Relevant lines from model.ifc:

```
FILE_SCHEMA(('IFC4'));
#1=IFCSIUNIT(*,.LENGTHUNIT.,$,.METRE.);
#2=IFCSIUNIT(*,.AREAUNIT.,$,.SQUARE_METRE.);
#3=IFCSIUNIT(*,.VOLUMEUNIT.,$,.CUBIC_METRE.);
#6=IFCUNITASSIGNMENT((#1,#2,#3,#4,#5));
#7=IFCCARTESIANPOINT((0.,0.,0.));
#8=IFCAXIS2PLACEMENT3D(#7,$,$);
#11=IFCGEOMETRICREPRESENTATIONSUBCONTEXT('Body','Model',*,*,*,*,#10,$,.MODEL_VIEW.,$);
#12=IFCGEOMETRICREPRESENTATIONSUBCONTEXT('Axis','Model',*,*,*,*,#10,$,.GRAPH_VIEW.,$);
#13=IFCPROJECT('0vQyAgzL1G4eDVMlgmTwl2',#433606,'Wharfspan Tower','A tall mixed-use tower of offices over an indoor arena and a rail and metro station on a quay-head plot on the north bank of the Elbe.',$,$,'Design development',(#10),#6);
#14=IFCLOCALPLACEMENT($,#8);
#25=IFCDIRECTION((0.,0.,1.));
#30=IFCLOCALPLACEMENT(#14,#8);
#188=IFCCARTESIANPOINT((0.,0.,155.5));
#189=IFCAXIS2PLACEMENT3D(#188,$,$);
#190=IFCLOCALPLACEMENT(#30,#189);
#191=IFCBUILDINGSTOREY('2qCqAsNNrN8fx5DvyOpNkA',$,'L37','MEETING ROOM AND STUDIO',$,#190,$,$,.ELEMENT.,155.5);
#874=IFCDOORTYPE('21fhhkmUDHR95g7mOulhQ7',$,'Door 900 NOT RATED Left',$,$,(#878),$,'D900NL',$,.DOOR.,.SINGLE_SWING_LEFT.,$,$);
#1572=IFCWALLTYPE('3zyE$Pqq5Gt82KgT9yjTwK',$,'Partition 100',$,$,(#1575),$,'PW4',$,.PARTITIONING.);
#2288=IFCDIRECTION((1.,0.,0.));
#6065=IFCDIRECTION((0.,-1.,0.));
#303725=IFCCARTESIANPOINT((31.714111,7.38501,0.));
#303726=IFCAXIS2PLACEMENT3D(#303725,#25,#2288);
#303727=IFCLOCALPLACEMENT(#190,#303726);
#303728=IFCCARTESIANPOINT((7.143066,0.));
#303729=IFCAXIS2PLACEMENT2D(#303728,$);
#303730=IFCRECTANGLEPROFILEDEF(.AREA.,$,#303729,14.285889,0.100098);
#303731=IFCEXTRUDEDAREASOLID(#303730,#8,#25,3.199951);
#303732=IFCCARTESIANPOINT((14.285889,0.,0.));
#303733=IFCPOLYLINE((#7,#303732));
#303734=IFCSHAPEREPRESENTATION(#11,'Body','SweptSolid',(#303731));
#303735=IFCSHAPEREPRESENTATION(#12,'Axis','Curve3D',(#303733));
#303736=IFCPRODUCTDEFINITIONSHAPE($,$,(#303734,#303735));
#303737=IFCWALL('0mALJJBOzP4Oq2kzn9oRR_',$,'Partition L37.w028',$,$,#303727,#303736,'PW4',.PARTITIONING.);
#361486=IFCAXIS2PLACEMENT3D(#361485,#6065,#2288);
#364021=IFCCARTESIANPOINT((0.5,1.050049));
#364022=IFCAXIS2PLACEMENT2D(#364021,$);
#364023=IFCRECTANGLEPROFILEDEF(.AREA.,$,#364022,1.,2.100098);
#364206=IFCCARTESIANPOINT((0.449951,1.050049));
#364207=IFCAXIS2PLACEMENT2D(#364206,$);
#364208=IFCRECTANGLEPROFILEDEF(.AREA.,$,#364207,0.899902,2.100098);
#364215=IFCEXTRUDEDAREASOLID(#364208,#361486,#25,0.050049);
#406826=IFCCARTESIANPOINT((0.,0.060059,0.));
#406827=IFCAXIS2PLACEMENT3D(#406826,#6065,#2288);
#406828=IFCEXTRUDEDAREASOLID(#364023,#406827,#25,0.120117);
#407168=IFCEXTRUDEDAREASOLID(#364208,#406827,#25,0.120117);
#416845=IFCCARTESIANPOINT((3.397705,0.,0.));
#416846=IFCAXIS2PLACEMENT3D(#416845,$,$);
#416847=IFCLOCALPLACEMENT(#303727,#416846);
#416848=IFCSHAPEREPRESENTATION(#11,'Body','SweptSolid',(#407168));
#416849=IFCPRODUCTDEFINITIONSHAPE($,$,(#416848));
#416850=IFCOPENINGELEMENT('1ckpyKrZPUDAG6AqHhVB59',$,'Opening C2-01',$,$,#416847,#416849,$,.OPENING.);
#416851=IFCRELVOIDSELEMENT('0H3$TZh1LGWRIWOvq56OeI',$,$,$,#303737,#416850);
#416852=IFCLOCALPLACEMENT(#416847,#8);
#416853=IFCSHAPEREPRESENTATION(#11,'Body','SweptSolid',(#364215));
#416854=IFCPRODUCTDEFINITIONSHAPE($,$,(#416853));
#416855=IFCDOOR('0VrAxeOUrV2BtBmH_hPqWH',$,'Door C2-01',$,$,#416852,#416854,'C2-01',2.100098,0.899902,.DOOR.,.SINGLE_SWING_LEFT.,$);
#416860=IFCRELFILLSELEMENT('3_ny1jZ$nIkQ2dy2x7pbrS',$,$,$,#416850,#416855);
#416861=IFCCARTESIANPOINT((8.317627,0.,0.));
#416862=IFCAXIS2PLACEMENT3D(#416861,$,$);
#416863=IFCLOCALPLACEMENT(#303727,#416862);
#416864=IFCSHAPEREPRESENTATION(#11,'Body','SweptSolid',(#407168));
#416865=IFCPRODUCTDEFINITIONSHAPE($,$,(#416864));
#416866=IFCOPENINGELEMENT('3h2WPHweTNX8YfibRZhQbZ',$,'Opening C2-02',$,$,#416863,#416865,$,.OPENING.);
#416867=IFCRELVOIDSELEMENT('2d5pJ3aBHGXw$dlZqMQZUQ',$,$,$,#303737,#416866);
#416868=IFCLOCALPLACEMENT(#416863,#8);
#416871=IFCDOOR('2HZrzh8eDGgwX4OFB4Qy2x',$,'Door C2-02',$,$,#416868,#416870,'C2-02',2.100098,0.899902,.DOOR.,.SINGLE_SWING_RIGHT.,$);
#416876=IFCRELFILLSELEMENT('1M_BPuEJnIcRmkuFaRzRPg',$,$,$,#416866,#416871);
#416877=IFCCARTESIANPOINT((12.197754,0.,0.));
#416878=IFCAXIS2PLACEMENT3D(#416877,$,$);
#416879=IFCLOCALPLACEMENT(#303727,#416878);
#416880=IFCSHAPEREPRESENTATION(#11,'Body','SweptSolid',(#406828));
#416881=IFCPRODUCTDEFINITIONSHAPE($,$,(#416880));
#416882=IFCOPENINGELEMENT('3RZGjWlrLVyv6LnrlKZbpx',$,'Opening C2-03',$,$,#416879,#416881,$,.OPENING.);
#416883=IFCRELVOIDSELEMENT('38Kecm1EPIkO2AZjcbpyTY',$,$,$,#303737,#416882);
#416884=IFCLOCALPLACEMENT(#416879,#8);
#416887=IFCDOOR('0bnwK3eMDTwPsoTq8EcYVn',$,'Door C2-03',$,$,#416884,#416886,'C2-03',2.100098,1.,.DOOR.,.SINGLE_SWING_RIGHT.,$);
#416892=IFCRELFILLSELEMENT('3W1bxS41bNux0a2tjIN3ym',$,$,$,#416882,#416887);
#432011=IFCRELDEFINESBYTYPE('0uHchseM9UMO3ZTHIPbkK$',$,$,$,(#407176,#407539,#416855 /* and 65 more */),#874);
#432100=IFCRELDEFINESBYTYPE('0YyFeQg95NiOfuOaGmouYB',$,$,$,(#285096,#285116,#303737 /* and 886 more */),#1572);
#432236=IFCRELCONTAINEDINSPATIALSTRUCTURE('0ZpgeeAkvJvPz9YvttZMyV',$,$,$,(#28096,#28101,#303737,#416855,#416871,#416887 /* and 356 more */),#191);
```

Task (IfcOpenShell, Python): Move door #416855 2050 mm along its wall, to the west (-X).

```python
import ifcopenshell
import ifcopenshell.api.geometry
import ifcopenshell.util.placement
import ifcopenshell.util.unit

model = ifcopenshell.open("model.ifc")
unit_scale = ifcopenshell.util.unit.calculate_unit_scale(model)

door = model.by_guid("0VrAxeOUrV2BtBmH_hPqWH")
opening = door.FillsVoids[0].RelatingOpeningElement
wall = opening.VoidsElements[0].RelatingBuildingElement

wall_matrix = ifcopenshell.util.placement.get_local_placement(wall.ObjectPlacement)
shift = wall_matrix[:3, 0] * -2.05 / unit_scale
before = ifcopenshell.util.placement.get_local_placement(door.ObjectPlacement)[:3, 3].copy()

# The door is placed relative to its opening, so it follows when the opening moves.
matrix = ifcopenshell.util.placement.get_local_placement(opening.ObjectPlacement)
matrix[:3, 3] += shift
ifcopenshell.api.geometry.edit_object_placement(
    model, product=opening, matrix=matrix, is_si=False, should_transform_children=True
)

after = ifcopenshell.util.placement.get_local_placement(door.ObjectPlacement)[:3, 3]
print("door moved by", (after - before).round(3) + 0.0)

model.write("model_v2.ifc")
```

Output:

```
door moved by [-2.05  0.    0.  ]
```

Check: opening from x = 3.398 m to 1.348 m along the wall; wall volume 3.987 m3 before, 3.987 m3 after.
